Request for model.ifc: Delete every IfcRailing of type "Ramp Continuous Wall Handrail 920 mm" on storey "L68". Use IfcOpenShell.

First a look at what the model holds.

```python
import ifcopenshell
import ifcopenshell.util.element

model = ifcopenshell.open("model.ifc")
print(model.schema)
storey = next(s for s in model.by_type("IfcBuildingStorey") if s.Name == "L68")
railings = [e for e in ifcopenshell.util.element.get_decomposition(storey) if e.is_a("IfcRailing")]
seen = {}
for e in railings:
    element_type = ifcopenshell.util.element.get_type(e)
    name = element_type.Name if element_type not in (None, e) else None
    seen[name] = seen.get(name, 0) + 1
for name, count in sorted(seen.items(), key=str):
    print(count, "x", name)
```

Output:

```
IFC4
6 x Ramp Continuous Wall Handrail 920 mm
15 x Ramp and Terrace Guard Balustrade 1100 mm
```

```python
import ifcopenshell
import ifcopenshell.api.root
import ifcopenshell.util.element

model = ifcopenshell.open("model.ifc")

storey = next(s for s in model.by_type("IfcBuildingStorey") if s.Name == "L68")
railings = [e for e in ifcopenshell.util.element.get_decomposition(storey) if e.is_a("IfcRailing")]
targets = [e for e in railings if (t := ifcopenshell.util.element.get_type(e)) not in (None, e) and t.Name == "Ramp Continuous Wall Handrail 920 mm"]

for e in targets:
    ifcopenshell.api.root.remove_product(model, product=e)
print(len(targets), "removed")

model.write("model_edited.ifc")
```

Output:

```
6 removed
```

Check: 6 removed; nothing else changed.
